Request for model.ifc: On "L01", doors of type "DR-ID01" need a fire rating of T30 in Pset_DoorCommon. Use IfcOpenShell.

First a look at what the model holds.

```python
import ifcopenshell
import ifcopenshell.util.element

model = ifcopenshell.open("model.ifc")
print(model.schema)
storey = next(s for s in model.by_type("IfcBuildingStorey") if s.Name == "L01")
doors = [e for e in ifcopenshell.util.element.get_decomposition(storey) if e.is_a("IfcDoor")]
seen = {}
for e in doors:
    element_type = ifcopenshell.util.element.get_type(e)
    key = (element_type.Name if element_type != e and element_type else None, ifcopenshell.util.element.get_pset(e, "Pset_DoorCommon", "FireRating"))
    seen[key] = seen.get(key, 0) + 1
for (name, value), count in sorted(seen.items(), key=str):
    print(count, "x", name, "|", value)
```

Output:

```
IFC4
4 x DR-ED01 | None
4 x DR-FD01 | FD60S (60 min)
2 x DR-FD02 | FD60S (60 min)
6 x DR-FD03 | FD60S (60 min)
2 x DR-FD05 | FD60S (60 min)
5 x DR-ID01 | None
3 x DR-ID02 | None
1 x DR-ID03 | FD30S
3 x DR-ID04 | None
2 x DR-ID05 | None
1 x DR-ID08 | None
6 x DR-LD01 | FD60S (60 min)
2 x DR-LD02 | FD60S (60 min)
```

```python
import ifcopenshell
import ifcopenshell.api.pset
import ifcopenshell.util.element

model = ifcopenshell.open("model.ifc")

storey = next(s for s in model.by_type("IfcBuildingStorey") if s.Name == "L01")
doors = [e for e in ifcopenshell.util.element.get_decomposition(storey) if e.is_a("IfcDoor")]

count = 0
for e in doors:
    element_type = ifcopenshell.util.element.get_type(e)
    if element_type in (None, e) or element_type.Name != "DR-ID01":
        continue
    # add_pset returns the element's existing set when there is one.
    pset = ifcopenshell.api.pset.add_pset(model, product=e, name="Pset_DoorCommon")
    ifcopenshell.api.pset.edit_pset(model, pset=pset, properties={"FireRating": "T30"})
    count += 1

print(count, "doors updated")

model.write("model_updated.ifc")
```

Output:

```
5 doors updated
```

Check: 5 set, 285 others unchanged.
